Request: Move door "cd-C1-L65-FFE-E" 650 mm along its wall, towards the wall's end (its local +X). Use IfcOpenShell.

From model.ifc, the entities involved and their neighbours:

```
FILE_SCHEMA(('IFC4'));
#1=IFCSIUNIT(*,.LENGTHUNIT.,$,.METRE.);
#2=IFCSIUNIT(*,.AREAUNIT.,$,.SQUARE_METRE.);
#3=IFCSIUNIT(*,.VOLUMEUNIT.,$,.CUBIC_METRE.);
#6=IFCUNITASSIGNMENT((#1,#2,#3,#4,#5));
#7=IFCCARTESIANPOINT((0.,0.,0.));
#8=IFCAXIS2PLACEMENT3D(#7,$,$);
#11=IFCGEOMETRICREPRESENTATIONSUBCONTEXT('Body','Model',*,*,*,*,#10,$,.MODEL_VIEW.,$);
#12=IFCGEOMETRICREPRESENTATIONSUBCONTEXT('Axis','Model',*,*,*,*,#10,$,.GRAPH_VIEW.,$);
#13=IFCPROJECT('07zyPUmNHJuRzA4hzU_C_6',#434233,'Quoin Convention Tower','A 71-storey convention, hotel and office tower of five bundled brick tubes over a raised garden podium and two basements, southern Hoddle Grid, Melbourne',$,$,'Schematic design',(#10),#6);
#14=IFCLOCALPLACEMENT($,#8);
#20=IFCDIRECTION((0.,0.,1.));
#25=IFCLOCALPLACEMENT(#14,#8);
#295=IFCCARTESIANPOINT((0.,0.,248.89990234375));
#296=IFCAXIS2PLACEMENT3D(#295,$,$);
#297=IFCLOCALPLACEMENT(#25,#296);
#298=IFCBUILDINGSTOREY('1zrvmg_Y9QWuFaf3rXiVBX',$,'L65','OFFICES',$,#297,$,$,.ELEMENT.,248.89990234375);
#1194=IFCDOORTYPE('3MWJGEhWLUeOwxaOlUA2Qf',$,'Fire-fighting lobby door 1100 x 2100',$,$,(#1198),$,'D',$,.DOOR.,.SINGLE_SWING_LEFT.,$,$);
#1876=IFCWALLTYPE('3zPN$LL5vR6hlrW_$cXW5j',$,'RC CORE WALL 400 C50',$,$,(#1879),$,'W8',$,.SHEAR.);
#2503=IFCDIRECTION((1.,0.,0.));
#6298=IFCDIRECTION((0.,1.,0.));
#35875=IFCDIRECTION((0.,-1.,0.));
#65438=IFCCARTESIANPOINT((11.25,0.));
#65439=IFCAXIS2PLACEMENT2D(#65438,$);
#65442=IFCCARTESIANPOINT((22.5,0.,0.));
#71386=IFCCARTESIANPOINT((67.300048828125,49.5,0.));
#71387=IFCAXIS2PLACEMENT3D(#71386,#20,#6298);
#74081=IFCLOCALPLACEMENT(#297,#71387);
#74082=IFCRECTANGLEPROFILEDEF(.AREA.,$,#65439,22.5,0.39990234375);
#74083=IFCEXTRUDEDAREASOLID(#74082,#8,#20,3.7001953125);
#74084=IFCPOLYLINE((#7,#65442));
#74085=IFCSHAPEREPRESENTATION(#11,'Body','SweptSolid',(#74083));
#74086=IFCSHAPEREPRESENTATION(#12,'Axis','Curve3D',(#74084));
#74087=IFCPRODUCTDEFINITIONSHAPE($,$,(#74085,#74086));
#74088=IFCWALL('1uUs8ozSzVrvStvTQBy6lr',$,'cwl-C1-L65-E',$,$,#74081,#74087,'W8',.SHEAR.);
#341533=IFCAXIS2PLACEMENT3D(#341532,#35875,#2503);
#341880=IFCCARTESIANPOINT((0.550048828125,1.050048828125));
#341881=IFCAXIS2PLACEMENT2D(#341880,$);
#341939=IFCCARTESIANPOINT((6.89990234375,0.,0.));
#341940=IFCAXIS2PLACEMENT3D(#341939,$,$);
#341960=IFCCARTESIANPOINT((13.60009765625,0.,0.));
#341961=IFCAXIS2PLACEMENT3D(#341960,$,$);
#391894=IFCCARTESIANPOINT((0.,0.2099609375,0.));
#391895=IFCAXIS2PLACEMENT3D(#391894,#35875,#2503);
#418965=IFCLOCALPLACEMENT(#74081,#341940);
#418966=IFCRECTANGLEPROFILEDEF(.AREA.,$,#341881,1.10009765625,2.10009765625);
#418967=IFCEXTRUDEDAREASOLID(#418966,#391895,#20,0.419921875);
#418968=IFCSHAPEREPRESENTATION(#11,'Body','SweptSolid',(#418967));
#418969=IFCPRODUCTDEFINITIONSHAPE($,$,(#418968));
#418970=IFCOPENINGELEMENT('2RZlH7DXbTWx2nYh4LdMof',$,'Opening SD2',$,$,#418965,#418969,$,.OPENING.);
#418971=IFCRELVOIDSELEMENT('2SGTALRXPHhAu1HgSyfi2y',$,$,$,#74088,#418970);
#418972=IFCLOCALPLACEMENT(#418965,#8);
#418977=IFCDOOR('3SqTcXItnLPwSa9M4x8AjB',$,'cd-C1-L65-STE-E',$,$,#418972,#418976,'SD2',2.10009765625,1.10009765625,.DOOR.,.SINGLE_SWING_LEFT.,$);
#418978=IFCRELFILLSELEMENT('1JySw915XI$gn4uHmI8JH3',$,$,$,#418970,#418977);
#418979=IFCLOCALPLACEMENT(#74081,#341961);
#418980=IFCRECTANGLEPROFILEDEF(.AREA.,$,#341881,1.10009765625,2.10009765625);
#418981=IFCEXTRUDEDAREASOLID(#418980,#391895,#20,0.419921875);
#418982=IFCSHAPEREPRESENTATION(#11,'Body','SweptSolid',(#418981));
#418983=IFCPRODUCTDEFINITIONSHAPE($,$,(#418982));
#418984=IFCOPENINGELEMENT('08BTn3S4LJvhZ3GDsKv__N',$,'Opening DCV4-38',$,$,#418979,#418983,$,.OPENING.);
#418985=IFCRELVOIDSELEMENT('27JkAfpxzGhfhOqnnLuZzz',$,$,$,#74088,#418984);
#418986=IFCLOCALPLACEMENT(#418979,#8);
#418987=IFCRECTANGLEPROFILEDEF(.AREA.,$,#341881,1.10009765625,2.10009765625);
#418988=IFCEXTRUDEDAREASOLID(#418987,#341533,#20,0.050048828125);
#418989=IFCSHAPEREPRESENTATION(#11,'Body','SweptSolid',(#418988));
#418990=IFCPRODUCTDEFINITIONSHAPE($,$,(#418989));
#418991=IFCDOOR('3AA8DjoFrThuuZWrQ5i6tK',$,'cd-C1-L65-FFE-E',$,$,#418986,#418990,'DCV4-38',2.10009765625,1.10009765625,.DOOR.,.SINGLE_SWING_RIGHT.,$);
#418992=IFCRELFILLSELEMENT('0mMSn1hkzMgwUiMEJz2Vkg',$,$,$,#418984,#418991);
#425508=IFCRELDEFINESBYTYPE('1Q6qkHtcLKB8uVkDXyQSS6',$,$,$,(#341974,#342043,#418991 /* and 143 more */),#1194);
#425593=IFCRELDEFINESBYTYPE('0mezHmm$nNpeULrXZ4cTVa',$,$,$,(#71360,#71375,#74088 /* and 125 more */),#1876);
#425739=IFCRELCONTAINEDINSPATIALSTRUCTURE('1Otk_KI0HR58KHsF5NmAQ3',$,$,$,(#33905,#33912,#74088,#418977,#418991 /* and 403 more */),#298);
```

```python
import ifcopenshell
import ifcopenshell.api.geometry
import ifcopenshell.util.placement
import ifcopenshell.util.unit

model = ifcopenshell.open("model.ifc")
unit_scale = ifcopenshell.util.unit.calculate_unit_scale(model)

door = model.by_guid("3AA8DjoFrThuuZWrQ5i6tK")
opening = door.FillsVoids[0].RelatingOpeningElement
wall = opening.VoidsElements[0].RelatingBuildingElement

wall_matrix = ifcopenshell.util.placement.get_local_placement(wall.ObjectPlacement)
shift = wall_matrix[:3, 0] * 0.65 / unit_scale
before = ifcopenshell.util.placement.get_local_placement(door.ObjectPlacement)[:3, 3].copy()

# The door is placed relative to its opening, so it follows when the opening moves.
matrix = ifcopenshell.util.placement.get_local_placement(opening.ObjectPlacement)
matrix[:3, 3] += shift
ifcopenshell.api.geometry.edit_object_placement(
    model, product=opening, matrix=matrix, is_si=False, should_transform_children=True
)

after = ifcopenshell.util.placement.get_local_placement(door.ObjectPlacement)[:3, 3]
print("door moved by", (after - before).round(3) + 0.0)

model.write("model_updated.ifc")
```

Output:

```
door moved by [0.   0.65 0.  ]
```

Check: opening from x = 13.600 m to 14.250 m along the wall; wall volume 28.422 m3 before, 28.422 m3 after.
